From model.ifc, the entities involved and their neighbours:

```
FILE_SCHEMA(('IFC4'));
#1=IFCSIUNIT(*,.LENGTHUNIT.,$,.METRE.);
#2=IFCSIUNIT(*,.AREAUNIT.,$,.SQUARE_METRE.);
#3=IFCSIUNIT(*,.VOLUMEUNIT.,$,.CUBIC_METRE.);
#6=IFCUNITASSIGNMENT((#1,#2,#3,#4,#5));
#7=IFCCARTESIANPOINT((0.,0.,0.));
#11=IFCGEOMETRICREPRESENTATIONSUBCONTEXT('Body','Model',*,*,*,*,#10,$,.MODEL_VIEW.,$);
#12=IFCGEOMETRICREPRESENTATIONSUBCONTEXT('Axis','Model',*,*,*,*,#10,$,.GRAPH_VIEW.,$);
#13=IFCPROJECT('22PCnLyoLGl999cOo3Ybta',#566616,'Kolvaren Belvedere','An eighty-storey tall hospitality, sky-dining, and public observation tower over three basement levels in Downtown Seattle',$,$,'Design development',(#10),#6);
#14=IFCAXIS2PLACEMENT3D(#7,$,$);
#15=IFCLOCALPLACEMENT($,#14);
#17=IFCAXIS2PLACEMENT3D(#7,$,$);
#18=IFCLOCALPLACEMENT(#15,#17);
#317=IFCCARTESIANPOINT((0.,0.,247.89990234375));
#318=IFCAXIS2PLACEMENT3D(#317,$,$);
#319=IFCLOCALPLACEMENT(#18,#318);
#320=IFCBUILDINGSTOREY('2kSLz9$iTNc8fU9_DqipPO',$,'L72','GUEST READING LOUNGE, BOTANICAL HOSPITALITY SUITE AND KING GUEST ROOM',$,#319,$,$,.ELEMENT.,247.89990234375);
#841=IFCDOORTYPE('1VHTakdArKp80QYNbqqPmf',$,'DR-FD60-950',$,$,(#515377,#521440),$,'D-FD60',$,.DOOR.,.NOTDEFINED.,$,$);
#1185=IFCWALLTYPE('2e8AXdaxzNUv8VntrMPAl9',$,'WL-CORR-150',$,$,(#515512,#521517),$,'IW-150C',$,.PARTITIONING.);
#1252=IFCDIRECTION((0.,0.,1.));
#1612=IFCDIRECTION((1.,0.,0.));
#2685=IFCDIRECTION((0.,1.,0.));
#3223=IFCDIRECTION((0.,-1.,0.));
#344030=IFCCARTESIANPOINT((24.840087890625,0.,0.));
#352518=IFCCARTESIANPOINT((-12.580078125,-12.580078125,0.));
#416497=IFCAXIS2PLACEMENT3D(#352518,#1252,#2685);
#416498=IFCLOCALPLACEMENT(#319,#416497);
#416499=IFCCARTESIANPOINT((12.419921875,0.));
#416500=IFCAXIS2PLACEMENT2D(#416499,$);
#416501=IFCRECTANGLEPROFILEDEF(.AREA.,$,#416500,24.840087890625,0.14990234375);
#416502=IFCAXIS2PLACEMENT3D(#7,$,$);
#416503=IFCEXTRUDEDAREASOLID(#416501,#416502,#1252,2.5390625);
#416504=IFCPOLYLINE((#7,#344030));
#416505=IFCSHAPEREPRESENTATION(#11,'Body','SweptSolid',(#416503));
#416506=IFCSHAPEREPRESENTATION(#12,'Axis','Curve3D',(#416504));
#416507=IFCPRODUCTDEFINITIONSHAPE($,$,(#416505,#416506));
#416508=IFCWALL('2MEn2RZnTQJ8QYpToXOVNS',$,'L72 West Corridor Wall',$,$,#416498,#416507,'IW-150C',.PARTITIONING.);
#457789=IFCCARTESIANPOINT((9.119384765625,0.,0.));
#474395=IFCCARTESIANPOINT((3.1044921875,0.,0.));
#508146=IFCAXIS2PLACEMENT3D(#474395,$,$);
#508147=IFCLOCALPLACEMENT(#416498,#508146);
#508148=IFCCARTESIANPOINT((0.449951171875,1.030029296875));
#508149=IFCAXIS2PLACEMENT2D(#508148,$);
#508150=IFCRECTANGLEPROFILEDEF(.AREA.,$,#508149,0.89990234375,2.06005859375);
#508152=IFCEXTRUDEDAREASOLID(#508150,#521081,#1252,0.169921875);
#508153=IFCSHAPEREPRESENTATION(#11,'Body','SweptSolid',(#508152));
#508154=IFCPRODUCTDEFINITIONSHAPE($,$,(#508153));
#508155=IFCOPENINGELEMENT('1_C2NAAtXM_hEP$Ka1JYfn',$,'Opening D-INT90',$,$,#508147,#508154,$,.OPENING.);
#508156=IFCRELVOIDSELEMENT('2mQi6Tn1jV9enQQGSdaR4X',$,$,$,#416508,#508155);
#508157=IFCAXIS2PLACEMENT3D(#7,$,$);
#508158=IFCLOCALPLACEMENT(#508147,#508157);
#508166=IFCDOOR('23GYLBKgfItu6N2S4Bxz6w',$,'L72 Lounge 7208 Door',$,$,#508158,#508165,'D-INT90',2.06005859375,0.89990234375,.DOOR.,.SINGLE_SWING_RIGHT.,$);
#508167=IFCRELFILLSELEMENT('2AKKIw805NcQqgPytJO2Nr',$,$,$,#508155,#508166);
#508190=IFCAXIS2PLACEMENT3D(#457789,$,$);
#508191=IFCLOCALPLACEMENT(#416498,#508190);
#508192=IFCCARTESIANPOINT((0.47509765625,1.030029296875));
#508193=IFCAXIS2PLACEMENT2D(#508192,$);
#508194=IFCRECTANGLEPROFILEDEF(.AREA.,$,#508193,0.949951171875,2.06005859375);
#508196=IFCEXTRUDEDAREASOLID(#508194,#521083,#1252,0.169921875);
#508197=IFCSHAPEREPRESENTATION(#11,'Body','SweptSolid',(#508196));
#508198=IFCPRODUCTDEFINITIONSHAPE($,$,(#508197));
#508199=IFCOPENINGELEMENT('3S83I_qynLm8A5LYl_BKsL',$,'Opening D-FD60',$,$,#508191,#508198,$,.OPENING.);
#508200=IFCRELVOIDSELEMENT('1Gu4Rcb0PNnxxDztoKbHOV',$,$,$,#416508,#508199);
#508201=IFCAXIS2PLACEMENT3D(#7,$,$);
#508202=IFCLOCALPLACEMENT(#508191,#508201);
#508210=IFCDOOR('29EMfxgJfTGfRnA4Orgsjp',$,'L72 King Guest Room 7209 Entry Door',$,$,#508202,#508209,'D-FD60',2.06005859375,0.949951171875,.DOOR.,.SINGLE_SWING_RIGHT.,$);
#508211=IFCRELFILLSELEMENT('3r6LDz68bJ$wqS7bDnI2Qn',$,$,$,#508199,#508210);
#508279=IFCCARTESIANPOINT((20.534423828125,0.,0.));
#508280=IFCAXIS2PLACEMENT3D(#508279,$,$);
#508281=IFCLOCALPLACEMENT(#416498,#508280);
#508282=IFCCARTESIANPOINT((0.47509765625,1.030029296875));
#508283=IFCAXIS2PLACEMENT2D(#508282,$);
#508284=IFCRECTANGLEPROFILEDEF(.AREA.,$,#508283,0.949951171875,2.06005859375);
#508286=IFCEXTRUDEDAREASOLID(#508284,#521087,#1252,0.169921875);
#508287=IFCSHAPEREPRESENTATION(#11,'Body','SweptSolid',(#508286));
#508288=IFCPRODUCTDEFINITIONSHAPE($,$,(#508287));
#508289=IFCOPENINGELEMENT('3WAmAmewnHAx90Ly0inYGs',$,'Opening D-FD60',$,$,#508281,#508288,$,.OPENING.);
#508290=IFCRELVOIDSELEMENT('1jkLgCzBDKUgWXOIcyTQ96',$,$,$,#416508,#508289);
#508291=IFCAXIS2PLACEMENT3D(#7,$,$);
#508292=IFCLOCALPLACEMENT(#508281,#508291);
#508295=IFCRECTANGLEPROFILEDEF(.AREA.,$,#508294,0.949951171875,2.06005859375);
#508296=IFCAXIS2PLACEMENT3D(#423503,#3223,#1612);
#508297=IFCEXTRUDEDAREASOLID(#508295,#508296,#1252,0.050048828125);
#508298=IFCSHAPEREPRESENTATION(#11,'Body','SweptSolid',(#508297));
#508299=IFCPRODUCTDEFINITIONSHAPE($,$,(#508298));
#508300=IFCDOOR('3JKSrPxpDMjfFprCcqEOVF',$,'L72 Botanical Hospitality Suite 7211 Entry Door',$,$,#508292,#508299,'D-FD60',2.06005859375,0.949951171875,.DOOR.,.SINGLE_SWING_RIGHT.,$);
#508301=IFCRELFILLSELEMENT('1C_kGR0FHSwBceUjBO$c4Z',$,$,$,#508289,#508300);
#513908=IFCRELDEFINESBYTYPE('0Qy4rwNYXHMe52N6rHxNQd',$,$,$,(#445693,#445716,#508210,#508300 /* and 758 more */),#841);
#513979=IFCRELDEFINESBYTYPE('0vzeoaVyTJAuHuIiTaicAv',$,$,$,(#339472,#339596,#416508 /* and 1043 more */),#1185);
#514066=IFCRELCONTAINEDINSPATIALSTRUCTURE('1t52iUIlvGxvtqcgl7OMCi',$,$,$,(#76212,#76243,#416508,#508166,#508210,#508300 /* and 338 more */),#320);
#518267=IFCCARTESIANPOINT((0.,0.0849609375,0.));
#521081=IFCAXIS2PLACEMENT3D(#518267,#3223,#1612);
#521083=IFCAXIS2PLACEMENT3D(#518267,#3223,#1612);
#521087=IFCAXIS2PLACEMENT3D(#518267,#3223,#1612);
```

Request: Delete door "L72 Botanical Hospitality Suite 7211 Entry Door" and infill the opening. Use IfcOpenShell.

```python
import ifcopenshell
import ifcopenshell.api.feature
import ifcopenshell.api.root
import ifcopenshell.geom
import ifcopenshell.util.shape

model = ifcopenshell.open("model.ifc")
settings = ifcopenshell.geom.settings()


def volume(element):
    """Net volume in cubic metres, openings subtracted."""
    shape = ifcopenshell.geom.create_shape(settings, element)
    return ifcopenshell.util.shape.get_volume(shape.geometry)


door = model.by_guid("3JKSrPxpDMjfFprCcqEOVF")
opening = door.FillsVoids[0].RelatingOpeningElement
wall = opening.VoidsElements[0].RelatingBuildingElement
before = volume(wall)

ifcopenshell.api.root.remove_product(model, product=door)
ifcopenshell.api.feature.remove_feature(model, feature=opening)

after = volume(wall)

print(f"wall volume {before:.3f} -> {after:.3f} m3")

model.write("model_v2.ifc")
```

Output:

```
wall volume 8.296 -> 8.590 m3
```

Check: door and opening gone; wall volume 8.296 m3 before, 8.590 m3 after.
